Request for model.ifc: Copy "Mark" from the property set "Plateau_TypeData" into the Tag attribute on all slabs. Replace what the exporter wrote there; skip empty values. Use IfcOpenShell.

First a look at what the model holds.

```python
import ifcopenshell
import ifcopenshell.util.element

model = ifcopenshell.open("model.ifc")
print(model.schema)
slabs = model.by_type("IfcSlab")
print(len(slabs), "slabs")
for e in slabs[:8]:
    source = ifcopenshell.util.element.get_pset(e, "Plateau_TypeData", "Mark")
    target = e.Tag
    print(e.id(), repr(source), repr(target), sep=" | ")
```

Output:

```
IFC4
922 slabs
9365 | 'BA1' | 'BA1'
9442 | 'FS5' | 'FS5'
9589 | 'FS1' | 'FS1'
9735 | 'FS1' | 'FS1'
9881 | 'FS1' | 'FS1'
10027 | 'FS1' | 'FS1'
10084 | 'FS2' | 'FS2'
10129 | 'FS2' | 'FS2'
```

```python
import ifcopenshell
import ifcopenshell.util.element

model = ifcopenshell.open("model.ifc")

count = 0
for e in model.by_type("IfcSlab"):
    value = ifcopenshell.util.element.get_pset(e, "Plateau_TypeData", "Mark")
    current = e.Tag
    if not value or not value.strip() or current == value:
        continue
    e.Tag = value
    count += 1

print(count, "slabs updated")

model.write("model-out.ifc")
```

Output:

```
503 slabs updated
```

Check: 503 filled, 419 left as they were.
